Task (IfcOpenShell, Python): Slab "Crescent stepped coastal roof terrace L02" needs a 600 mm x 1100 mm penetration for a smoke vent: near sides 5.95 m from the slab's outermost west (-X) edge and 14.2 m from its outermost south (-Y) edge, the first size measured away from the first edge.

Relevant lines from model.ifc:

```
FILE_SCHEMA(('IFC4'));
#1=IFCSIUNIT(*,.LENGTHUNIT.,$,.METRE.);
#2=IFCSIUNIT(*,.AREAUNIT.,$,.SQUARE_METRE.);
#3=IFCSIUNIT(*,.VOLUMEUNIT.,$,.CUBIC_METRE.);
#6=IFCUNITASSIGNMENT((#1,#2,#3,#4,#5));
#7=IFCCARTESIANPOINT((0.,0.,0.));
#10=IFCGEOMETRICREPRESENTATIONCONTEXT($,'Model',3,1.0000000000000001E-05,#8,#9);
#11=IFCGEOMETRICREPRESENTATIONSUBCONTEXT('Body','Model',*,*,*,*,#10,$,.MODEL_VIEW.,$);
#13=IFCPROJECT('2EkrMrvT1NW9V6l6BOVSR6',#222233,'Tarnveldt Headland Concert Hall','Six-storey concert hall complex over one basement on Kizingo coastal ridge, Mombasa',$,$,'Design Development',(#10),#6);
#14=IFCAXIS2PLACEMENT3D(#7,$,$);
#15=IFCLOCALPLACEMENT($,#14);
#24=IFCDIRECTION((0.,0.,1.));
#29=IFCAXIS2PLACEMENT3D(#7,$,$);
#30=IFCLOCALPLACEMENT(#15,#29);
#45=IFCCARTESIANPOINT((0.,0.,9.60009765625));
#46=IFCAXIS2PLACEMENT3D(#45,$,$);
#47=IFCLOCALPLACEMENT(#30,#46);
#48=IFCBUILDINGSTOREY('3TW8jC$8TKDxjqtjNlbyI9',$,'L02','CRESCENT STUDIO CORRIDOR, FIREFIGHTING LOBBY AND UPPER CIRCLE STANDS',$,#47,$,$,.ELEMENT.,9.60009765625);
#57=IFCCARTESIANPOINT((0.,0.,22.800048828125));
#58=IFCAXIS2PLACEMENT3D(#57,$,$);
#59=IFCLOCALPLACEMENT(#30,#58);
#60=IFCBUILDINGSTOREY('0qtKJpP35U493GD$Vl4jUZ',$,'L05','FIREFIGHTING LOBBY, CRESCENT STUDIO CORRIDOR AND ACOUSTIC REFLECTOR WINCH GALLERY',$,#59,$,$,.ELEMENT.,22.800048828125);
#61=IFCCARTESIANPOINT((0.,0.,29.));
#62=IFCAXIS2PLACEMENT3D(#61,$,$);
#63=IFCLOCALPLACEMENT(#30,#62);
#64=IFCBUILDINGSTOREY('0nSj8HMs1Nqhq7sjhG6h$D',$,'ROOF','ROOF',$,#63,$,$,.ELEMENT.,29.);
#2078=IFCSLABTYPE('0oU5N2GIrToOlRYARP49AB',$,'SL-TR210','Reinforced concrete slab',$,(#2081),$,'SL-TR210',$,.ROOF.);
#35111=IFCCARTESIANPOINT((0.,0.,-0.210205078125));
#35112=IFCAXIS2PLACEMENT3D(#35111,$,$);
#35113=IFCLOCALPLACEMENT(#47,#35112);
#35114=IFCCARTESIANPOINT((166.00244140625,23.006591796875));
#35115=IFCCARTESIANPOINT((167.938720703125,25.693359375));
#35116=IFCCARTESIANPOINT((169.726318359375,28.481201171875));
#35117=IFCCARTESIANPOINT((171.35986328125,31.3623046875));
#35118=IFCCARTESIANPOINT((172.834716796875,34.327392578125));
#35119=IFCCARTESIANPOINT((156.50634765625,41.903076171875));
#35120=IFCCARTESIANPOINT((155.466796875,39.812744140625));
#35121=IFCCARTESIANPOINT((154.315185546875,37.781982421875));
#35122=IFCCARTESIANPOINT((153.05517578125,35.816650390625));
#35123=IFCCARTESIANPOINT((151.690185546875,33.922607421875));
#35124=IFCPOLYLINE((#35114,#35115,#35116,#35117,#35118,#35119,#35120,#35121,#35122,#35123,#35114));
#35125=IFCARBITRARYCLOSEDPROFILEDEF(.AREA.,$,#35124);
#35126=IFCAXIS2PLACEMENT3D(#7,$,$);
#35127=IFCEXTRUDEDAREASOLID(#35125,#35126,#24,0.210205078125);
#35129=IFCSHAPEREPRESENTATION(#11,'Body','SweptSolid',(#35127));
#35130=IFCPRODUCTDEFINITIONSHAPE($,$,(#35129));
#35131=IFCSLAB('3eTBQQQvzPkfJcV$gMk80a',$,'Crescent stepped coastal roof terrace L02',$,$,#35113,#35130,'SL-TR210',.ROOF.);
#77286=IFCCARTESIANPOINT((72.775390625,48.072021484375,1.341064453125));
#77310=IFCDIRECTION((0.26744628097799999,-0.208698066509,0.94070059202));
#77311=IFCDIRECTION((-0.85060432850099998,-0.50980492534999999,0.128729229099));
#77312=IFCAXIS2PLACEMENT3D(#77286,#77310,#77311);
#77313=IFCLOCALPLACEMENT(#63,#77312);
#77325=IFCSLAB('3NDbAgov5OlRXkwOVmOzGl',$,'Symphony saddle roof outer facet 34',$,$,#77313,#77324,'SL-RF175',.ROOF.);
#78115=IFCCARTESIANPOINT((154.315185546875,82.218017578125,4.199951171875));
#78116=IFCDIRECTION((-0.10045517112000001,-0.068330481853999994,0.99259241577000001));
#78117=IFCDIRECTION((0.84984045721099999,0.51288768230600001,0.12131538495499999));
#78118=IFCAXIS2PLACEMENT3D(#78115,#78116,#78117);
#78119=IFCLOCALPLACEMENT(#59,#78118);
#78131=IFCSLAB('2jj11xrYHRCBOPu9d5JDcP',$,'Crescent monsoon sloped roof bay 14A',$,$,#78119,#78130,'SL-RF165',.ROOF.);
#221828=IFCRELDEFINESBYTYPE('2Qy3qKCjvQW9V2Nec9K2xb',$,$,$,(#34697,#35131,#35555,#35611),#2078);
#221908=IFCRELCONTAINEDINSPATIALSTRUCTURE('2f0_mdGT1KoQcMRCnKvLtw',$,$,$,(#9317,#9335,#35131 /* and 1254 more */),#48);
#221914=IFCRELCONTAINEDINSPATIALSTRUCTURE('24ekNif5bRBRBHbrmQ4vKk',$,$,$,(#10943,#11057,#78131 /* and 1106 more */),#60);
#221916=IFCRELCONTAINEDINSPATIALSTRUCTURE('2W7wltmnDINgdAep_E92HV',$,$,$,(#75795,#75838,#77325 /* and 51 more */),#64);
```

```python
import numpy as np
import ifcopenshell
import ifcopenshell.api.feature
import ifcopenshell.api.geometry
import ifcopenshell.api.root
import ifcopenshell.geom
import ifcopenshell.util.placement
import ifcopenshell.util.representation
import ifcopenshell.util.shape
import ifcopenshell.util.unit

model = ifcopenshell.open("model.ifc")
unit_scale = ifcopenshell.util.unit.calculate_unit_scale(model)
settings = ifcopenshell.geom.settings()


def volume(element):
    """Net volume in cubic metres, openings subtracted."""
    shape = ifcopenshell.geom.create_shape(settings, element)
    return ifcopenshell.util.shape.get_volume(shape.geometry)


slab = model.by_id(35131)
before = volume(slab)

# Extent in the slab's own axes, in metres. The edges named are its -X and -Y sides.
slab_shape = ifcopenshell.geom.create_shape(settings, slab)
vertices = ifcopenshell.util.shape.get_vertices(slab_shape.geometry)
x_min, y_min, bottom = vertices.min(axis=0)
top = vertices[:, 2].max()

opening = ifcopenshell.api.root.create_entity(model, ifc_class="IfcOpeningElement", name="Smoke vent opening", predefined_type="OPENING")
context = ifcopenshell.util.representation.get_context(model, "Model", "Body", "MODEL_VIEW")
width, depth = 0.6, 1.1
outline = [(0.0, 0.0), (width, 0.0), (width, depth), (0.0, depth), (0.0, 0.0)]
# Overshoot both faces by 50 mm so the cut is clean.
shape = ifcopenshell.api.geometry.add_slab_representation(
    model, context=context, depth=top - bottom + 0.1, polyline=outline
)
ifcopenshell.api.geometry.assign_representation(model, product=opening, representation=shape)

matrix = ifcopenshell.util.placement.get_local_placement(slab.ObjectPlacement)
matrix[:, 3] = matrix @ np.append(np.array([x_min + 5.95, y_min + 14.2, bottom - 0.05]) / unit_scale, 1.0)
ifcopenshell.api.geometry.edit_object_placement(model, product=opening, matrix=matrix, is_si=False)
ifcopenshell.api.feature.add_feature(model, feature=opening, element=slab)

after = volume(slab)

print(f"slab volume {before:.3f} -> {after:.3f} m3")

model.write("model_edited.ifc")
```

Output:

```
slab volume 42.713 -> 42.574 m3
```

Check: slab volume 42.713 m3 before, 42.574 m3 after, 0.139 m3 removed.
